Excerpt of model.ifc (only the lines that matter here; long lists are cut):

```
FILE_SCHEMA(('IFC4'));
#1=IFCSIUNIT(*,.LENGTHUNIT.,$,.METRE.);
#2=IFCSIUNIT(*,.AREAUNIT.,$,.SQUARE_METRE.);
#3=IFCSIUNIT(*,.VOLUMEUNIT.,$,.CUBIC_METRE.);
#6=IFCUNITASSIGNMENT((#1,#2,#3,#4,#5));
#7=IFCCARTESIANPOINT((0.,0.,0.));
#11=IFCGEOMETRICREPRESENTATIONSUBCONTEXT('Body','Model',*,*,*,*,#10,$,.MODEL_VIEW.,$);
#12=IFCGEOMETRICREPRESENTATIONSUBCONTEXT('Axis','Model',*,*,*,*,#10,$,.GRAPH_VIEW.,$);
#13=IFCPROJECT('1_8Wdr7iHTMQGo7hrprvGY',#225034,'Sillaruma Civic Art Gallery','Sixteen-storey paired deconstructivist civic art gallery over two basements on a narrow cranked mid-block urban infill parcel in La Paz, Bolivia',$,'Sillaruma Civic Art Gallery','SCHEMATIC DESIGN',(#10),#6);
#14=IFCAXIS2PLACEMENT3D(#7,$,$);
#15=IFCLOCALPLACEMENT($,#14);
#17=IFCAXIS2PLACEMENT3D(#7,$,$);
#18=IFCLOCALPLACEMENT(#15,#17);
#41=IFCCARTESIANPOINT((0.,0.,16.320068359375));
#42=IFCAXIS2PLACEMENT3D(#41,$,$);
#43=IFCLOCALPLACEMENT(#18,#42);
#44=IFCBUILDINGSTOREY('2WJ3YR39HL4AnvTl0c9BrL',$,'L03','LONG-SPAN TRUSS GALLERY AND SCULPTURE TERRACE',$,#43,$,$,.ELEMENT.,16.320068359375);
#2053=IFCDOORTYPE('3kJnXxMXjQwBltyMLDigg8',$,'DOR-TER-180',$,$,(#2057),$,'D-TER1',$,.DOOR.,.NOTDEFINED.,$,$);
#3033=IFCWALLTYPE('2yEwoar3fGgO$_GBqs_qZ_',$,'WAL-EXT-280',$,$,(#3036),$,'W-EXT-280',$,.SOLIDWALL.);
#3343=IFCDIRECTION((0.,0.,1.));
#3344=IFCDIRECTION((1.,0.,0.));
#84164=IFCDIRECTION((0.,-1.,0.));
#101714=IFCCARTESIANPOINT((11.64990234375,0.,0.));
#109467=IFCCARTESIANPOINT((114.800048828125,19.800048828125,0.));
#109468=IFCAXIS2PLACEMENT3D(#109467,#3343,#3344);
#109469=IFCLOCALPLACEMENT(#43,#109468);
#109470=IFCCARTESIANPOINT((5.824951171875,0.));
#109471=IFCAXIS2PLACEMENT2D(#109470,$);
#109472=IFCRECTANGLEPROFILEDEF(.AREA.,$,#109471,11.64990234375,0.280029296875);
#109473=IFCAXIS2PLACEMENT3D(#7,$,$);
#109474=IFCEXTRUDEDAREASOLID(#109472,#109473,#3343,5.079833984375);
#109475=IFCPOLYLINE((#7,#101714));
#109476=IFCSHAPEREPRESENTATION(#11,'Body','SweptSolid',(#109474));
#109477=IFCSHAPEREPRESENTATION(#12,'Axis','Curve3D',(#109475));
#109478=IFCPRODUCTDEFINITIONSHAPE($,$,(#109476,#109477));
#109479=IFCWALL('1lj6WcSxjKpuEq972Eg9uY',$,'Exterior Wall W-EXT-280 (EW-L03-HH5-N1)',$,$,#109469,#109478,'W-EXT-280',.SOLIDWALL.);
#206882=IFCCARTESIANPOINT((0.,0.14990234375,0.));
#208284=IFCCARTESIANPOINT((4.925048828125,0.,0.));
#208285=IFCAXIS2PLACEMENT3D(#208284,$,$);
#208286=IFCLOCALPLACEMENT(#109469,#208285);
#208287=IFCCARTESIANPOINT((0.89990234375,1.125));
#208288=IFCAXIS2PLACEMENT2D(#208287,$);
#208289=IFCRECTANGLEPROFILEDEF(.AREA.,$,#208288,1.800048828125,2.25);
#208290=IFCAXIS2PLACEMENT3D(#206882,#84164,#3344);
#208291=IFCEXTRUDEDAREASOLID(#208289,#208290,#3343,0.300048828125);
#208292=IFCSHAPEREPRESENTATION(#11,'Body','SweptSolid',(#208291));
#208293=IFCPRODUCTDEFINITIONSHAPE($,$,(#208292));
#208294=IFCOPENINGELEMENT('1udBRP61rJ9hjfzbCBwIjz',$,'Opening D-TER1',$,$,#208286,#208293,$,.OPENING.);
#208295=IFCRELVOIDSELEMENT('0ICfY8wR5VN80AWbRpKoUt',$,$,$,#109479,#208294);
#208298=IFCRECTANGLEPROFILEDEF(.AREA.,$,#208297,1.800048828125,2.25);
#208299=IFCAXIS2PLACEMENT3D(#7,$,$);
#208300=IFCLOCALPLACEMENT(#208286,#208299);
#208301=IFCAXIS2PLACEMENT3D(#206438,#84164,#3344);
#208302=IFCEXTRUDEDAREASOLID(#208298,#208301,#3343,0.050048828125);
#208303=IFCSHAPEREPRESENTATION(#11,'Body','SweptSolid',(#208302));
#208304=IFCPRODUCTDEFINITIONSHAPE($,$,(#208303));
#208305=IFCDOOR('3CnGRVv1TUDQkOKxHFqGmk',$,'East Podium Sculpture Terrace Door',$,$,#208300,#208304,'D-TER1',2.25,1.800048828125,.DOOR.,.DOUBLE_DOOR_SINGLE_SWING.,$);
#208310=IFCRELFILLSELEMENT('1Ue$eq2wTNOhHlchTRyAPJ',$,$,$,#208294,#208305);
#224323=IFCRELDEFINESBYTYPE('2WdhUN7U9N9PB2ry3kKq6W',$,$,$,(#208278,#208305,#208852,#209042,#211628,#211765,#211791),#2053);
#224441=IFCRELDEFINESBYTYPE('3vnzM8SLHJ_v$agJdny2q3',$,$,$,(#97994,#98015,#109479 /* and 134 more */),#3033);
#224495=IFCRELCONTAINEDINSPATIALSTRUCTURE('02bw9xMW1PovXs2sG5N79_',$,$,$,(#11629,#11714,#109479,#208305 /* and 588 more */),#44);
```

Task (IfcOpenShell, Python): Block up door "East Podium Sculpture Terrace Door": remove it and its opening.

```python
import ifcopenshell
import ifcopenshell.api.feature
import ifcopenshell.api.root
import ifcopenshell.geom
import ifcopenshell.util.shape

model = ifcopenshell.open("model.ifc")
settings = ifcopenshell.geom.settings()


def volume(element):
    """Net volume in cubic metres, openings subtracted."""
    shape = ifcopenshell.geom.create_shape(settings, element)
    return ifcopenshell.util.shape.get_volume(shape.geometry)


door = model.by_guid("3CnGRVv1TUDQkOKxHFqGmk")
opening = door.FillsVoids[0].RelatingOpeningElement
wall = opening.VoidsElements[0].RelatingBuildingElement
before = volume(wall)

ifcopenshell.api.root.remove_product(model, product=door)
ifcopenshell.api.feature.remove_feature(model, feature=opening)

after = volume(wall)

print(f"wall volume {before:.3f} -> {after:.3f} m3")

model.write("model_v2.ifc")
```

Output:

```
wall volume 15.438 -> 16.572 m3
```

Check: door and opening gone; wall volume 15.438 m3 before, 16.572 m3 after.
